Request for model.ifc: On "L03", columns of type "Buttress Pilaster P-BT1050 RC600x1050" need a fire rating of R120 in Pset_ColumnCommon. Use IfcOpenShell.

First a look at what the model holds.

```python
import ifcopenshell
import ifcopenshell.util.element

model = ifcopenshell.open("model.ifc")
print(model.schema)
storey = next(s for s in model.by_type("IfcBuildingStorey") if s.Name == "L03")
columns = [e for e in ifcopenshell.util.element.get_decomposition(storey) if e.is_a("IfcColumn")]
seen = {}
for e in columns:
    element_type = ifcopenshell.util.element.get_type(e)
    key = (element_type.Name if element_type != e and element_type else None, ifcopenshell.util.element.get_pset(e, "Pset_ColumnCommon", "FireRating"))
    seen[key] = seen.get(key, 0) + 1
for (name, value), count in sorted(seen.items(), key=str):
    print(count, "x", name, "|", value)
```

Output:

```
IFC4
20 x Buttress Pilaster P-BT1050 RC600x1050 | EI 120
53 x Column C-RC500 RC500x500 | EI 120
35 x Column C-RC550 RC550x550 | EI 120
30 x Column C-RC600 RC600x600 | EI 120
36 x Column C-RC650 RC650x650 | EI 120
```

```python
import ifcopenshell
import ifcopenshell.api.pset
import ifcopenshell.util.element

model = ifcopenshell.open("model.ifc")

storey = next(s for s in model.by_type("IfcBuildingStorey") if s.Name == "L03")
columns = [e for e in ifcopenshell.util.element.get_decomposition(storey) if e.is_a("IfcColumn")]

count = 0
for e in columns:
    element_type = ifcopenshell.util.element.get_type(e)
    if element_type in (None, e) or element_type.Name != "Buttress Pilaster P-BT1050 RC600x1050":
        continue
    # add_pset returns the element's existing set when there is one.
    pset = ifcopenshell.api.pset.add_pset(model, product=e, name="Pset_ColumnCommon")
    ifcopenshell.api.pset.edit_pset(model, pset=pset, properties={"FireRating": "R120"})
    count += 1

print(count, "columns updated")

model.write("model_edited.ifc")
```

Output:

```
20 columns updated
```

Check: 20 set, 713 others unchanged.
